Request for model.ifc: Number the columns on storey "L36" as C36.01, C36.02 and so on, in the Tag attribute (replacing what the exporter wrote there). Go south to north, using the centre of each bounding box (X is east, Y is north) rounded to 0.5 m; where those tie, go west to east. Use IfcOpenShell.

First a look at what the model holds.

```python
import ifcopenshell
import ifcopenshell.util.element
import ifcopenshell.util.placement

model = ifcopenshell.open("model.ifc")
print(model.schema)
storey = next(s for s in model.by_type("IfcBuildingStorey") if s.Name == "L36")
columns = [e for e in ifcopenshell.util.element.get_decomposition(storey) if e.is_a("IfcColumn")]
for e in sorted(columns, key=lambda e: e.id()):
    origin = ifcopenshell.util.placement.get_local_placement(e.ObjectPlacement)[:3, 3]
    print(e.id(), e.Tag, e.Name, origin.round(2) + 0.0, sep=" | ")
```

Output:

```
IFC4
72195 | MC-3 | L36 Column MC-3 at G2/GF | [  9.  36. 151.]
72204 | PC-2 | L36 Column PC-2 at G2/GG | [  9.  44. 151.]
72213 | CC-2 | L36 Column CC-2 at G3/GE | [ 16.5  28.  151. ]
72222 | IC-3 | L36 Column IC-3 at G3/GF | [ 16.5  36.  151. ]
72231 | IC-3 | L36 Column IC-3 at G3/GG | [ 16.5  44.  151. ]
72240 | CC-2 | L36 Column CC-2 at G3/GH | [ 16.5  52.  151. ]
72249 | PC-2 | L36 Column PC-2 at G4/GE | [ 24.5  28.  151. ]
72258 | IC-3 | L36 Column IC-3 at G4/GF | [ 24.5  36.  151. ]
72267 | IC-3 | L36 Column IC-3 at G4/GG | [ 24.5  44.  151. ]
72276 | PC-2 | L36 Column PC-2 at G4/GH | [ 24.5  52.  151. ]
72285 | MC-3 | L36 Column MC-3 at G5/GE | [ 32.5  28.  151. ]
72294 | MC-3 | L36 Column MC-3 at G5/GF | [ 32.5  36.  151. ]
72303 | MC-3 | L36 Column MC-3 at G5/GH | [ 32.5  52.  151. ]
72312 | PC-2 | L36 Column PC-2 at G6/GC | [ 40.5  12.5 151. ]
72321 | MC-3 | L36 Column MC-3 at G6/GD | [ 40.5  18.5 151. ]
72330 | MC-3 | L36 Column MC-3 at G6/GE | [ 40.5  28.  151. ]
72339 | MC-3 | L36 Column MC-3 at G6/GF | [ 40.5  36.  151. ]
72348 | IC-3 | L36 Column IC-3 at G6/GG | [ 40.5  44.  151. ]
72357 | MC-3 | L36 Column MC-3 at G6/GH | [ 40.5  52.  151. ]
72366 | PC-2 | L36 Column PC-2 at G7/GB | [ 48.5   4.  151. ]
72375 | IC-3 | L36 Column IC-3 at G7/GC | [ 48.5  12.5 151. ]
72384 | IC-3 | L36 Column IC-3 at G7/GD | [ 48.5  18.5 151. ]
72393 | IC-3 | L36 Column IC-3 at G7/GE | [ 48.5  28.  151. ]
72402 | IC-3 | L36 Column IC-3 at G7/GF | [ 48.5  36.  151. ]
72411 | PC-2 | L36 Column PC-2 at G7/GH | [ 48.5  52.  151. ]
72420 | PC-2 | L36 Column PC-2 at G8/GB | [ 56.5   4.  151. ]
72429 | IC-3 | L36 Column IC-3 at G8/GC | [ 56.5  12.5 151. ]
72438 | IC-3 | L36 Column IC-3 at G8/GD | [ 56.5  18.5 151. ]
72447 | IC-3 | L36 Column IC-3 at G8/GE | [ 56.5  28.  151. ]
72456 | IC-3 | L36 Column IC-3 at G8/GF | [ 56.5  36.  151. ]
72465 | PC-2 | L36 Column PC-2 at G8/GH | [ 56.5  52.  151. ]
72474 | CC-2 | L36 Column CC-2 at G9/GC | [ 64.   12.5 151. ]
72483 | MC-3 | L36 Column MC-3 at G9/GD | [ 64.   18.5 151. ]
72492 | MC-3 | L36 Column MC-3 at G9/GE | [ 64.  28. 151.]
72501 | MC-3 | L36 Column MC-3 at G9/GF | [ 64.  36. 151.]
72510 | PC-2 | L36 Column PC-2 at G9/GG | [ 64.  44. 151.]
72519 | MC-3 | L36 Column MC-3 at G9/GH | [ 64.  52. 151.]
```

```python
import ifcopenshell
import ifcopenshell.geom
import ifcopenshell.util.element
import ifcopenshell.util.shape

model = ifcopenshell.open("model.ifc")
settings = ifcopenshell.geom.settings()
settings.set("use-world-coords", True)


def centre(element):
    shape = ifcopenshell.geom.create_shape(settings, element)
    return ifcopenshell.util.shape.get_bbox_centroid(shape.geometry)


storey = next(s for s in model.by_type("IfcBuildingStorey") if s.Name == "L36")
columns = [e for e in ifcopenshell.util.element.get_decomposition(storey) if e.is_a("IfcColumn")]

# Insertion points can sit at a corner or the storey origin, so sort by the geometry (in metres).
centres = {e: centre(e) for e in columns}
columns.sort(key=lambda e: (round(centres[e][1] / 0.5), centres[e][0]))

for i, e in enumerate(columns, start=1):
    number = f"C36.{i:02d}"
    e.Tag = number
    print(e.id(), number)

model.write("model_rev.ifc")
```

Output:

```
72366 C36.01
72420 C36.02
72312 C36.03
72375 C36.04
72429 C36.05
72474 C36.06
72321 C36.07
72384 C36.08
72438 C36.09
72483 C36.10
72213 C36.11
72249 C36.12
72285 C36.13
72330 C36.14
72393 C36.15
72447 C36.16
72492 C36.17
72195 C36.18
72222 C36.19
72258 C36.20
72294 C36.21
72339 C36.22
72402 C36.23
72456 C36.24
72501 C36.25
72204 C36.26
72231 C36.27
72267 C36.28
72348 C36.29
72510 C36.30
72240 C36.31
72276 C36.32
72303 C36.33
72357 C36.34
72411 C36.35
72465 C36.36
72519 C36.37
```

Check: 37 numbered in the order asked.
